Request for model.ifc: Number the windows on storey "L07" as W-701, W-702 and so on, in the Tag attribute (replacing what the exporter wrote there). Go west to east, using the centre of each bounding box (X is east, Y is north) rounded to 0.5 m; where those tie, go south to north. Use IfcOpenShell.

First a look at what the model holds.

```python
import ifcopenshell
import ifcopenshell.util.element
import ifcopenshell.util.placement

model = ifcopenshell.open("model.ifc")
print(model.schema)
storey = next(s for s in model.by_type("IfcBuildingStorey") if s.Name == "L07")
windows = [e for e in ifcopenshell.util.element.get_decomposition(storey) if e.is_a("IfcWindow")]
for e in sorted(windows, key=lambda e: e.id()):
    origin = ifcopenshell.util.placement.get_local_placement(e.ObjectPlacement)[:3, 3]
    print(e.id(), e.Tag, e.Name, origin.round(2) + 0.0, sep=" | ")
```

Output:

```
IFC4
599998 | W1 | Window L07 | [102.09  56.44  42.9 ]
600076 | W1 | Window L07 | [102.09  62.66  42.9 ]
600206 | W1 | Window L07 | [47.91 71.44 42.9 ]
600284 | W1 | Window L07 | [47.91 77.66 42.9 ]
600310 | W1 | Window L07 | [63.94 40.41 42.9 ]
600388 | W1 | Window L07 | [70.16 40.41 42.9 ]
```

```python
import ifcopenshell
import ifcopenshell.geom
import ifcopenshell.util.element
import ifcopenshell.util.shape

model = ifcopenshell.open("model.ifc")
settings = ifcopenshell.geom.settings()
settings.set("use-world-coords", True)


def centre(element):
    shape = ifcopenshell.geom.create_shape(settings, element)
    return ifcopenshell.util.shape.get_bbox_centroid(shape.geometry)


storey = next(s for s in model.by_type("IfcBuildingStorey") if s.Name == "L07")
windows = [e for e in ifcopenshell.util.element.get_decomposition(storey) if e.is_a("IfcWindow")]

# Insertion points can sit at a corner or the storey origin, so sort by the geometry (in metres).
centres = {e: centre(e) for e in windows}
windows.sort(key=lambda e: (round(centres[e][0] / 0.5), centres[e][1]))

for i, e in enumerate(windows, start=1):
    number = f"W-7{i:02d}"
    e.Tag = number
    print(e.id(), number)

model.write("model-out.ifc")
```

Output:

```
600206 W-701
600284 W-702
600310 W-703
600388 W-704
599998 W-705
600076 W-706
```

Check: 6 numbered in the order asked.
